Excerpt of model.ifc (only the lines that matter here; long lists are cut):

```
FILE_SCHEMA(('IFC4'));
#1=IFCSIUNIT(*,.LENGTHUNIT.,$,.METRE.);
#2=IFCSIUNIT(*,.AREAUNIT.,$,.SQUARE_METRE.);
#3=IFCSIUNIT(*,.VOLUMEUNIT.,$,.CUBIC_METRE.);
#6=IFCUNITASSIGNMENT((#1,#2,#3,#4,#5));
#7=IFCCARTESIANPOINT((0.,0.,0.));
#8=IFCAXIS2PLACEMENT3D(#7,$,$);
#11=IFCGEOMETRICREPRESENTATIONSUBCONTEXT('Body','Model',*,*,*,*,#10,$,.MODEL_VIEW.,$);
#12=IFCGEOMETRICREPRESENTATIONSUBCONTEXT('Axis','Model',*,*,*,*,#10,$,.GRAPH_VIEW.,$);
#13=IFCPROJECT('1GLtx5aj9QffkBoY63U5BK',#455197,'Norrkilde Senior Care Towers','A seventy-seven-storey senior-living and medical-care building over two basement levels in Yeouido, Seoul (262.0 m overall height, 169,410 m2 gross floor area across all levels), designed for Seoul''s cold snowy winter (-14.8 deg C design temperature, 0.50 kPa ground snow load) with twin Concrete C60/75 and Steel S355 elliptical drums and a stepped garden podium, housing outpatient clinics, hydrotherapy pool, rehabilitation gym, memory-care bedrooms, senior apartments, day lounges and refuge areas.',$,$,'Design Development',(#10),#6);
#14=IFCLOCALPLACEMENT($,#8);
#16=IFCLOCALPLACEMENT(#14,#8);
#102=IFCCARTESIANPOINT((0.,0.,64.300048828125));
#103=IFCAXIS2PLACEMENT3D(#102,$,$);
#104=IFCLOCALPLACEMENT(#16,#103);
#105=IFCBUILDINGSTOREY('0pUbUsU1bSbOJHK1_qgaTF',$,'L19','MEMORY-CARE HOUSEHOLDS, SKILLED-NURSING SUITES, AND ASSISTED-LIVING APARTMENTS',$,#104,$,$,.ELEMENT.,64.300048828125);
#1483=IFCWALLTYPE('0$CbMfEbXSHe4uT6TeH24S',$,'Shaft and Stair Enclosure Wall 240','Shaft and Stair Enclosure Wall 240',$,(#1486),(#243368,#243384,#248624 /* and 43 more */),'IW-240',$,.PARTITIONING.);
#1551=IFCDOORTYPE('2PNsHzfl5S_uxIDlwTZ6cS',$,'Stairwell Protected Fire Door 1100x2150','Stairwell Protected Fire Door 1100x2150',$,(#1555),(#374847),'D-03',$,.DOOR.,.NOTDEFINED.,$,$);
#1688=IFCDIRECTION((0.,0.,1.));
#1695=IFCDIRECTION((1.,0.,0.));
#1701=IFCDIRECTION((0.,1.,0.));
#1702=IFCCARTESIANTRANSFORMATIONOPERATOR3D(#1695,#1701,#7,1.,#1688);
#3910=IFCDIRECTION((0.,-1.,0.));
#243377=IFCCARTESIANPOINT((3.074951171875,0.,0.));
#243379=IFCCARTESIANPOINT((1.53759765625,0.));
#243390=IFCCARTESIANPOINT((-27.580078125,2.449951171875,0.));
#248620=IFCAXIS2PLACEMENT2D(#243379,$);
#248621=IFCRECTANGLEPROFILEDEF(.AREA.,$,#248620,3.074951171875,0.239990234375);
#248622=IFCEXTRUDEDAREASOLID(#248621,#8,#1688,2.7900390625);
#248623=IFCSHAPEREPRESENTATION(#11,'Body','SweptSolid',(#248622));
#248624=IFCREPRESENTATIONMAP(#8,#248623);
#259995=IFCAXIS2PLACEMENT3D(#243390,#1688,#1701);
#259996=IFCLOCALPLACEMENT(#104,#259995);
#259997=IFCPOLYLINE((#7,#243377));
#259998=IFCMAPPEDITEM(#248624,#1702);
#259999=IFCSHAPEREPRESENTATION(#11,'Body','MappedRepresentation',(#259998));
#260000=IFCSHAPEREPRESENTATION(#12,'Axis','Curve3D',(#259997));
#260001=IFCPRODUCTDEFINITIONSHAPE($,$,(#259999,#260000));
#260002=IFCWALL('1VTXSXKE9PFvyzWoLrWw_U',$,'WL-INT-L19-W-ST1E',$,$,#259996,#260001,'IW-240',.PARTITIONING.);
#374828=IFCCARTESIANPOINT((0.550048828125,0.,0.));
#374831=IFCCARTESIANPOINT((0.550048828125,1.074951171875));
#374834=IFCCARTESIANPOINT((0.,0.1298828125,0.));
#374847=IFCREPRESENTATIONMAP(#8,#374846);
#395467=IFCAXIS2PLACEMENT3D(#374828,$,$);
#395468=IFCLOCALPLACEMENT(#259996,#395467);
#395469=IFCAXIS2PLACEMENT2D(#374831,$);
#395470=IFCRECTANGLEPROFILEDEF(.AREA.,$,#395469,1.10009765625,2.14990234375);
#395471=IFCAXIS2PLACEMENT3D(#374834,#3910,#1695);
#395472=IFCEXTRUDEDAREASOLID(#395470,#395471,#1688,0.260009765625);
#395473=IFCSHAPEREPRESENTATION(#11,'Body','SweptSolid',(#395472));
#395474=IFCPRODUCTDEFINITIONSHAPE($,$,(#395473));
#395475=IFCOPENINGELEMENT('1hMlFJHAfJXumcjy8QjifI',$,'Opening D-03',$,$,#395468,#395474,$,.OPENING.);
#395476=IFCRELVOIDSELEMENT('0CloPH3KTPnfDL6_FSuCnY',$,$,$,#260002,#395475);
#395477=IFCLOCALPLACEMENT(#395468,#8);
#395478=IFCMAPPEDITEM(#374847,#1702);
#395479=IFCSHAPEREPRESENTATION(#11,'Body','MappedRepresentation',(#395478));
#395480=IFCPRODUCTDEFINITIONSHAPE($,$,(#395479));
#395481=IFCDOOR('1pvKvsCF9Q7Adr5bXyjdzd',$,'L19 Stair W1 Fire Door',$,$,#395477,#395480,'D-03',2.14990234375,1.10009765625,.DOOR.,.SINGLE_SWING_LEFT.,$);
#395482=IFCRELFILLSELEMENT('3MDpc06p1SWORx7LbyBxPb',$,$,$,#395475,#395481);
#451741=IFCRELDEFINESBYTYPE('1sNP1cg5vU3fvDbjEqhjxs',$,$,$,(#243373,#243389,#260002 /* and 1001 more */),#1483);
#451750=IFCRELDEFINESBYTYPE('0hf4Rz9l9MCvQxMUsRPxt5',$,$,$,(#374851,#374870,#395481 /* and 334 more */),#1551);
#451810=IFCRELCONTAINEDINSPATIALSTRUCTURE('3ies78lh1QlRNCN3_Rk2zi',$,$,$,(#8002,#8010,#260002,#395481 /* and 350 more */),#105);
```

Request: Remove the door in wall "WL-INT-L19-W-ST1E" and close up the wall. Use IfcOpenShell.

```python
import ifcopenshell
import ifcopenshell.api.feature
import ifcopenshell.api.root
import ifcopenshell.geom
import ifcopenshell.util.shape

model = ifcopenshell.open("model.ifc")
settings = ifcopenshell.geom.settings()


def volume(element):
    """Net volume in cubic metres, openings subtracted."""
    shape = ifcopenshell.geom.create_shape(settings, element)
    return ifcopenshell.util.shape.get_volume(shape.geometry)


door = model.by_guid("1pvKvsCF9Q7Adr5bXyjdzd")
opening = door.FillsVoids[0].RelatingOpeningElement
wall = opening.VoidsElements[0].RelatingBuildingElement
before = volume(wall)

ifcopenshell.api.root.remove_product(model, product=door)
ifcopenshell.api.feature.remove_feature(model, feature=opening)

after = volume(wall)

print(f"wall volume {before:.3f} -> {after:.3f} m3")

model.write("model_edited.ifc")
```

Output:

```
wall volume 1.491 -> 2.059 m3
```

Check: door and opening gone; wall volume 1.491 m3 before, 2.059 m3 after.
